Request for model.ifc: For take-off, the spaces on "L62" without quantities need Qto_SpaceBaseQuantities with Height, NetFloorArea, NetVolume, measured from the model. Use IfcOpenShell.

First a look at what the model holds.

```python
import ifcopenshell
import ifcopenshell.util.element
import ifcopenshell.util.unit

model = ifcopenshell.open("model.ifc")
print(model.schema)
for unit_type in ("LENGTHUNIT", "AREAUNIT", "VOLUMEUNIT"):
    print(unit_type, ifcopenshell.util.unit.calculate_unit_scale(model, unit_type))
storey = next(s for s in model.by_type("IfcBuildingStorey") if s.Name == "L62")
spaces = [e for e in ifcopenshell.util.element.get_decomposition(storey) if e.is_a("IfcSpace")]
for e in sorted(spaces, key=lambda e: e.id()):
    print(e.id(), e.is_a(), e.Name, list(ifcopenshell.util.element.get_psets(e, qtos_only=True)), sep=" | ")
```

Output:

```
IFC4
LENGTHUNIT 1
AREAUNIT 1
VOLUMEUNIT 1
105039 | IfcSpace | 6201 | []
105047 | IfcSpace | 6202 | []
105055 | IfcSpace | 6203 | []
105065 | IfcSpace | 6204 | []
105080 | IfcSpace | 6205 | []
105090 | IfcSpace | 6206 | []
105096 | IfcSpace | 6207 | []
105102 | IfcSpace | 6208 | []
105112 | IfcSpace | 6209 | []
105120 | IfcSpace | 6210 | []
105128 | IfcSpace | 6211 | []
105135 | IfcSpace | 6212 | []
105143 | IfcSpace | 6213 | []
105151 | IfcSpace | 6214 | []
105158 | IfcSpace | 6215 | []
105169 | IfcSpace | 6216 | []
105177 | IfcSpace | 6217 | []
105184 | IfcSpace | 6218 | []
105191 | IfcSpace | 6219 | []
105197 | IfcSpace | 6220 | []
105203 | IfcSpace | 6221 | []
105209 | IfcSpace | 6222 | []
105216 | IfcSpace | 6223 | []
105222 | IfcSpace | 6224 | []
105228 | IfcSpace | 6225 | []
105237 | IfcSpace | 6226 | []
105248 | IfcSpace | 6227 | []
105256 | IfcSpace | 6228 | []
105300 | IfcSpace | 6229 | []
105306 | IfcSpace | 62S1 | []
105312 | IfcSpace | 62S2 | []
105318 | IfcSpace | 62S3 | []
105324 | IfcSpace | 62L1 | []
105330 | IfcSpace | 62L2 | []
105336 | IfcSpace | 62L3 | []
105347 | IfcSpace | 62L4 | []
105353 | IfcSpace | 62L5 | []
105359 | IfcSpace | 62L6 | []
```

```python
import ifcopenshell
import ifcopenshell.api.pset
import ifcopenshell.geom
import ifcopenshell.util.element
import ifcopenshell.util.shape
import ifcopenshell.util.unit

model = ifcopenshell.open("model.ifc")
unit_scale = ifcopenshell.util.unit.calculate_unit_scale(model)
area_scale = ifcopenshell.util.unit.calculate_unit_scale(model, "AREAUNIT")
volume_scale = ifcopenshell.util.unit.calculate_unit_scale(model, "VOLUMEUNIT")
settings = ifcopenshell.geom.settings()

storey = next(s for s in model.by_type("IfcBuildingStorey") if s.Name == "L62")
spaces = [e for e in ifcopenshell.util.element.get_decomposition(storey) if e.is_a("IfcSpace")]

for e in sorted(spaces, key=lambda e: e.id()):
    if ifcopenshell.util.element.get_psets(e, qtos_only=True, should_inherit=False):
        continue
    # Geometry comes back in metres, in the element's own axes.
    shape = ifcopenshell.geom.create_shape(settings, e)
    values = {
        "Height": ifcopenshell.util.shape.get_z(shape.geometry) / unit_scale,
        "NetFloorArea": ifcopenshell.util.shape.get_footprint_area(shape.geometry) / area_scale,
        "NetVolume": ifcopenshell.util.shape.get_volume(shape.geometry) / volume_scale,
    }
    qto = ifcopenshell.api.pset.add_qto(model, product=e, name="Qto_SpaceBaseQuantities")
    ifcopenshell.api.pset.edit_qto(model, qto=qto, properties=values)
    print(e.id(), {k: round(v, 3) for k, v in values.items()})

model.write("model_v2.ifc")
```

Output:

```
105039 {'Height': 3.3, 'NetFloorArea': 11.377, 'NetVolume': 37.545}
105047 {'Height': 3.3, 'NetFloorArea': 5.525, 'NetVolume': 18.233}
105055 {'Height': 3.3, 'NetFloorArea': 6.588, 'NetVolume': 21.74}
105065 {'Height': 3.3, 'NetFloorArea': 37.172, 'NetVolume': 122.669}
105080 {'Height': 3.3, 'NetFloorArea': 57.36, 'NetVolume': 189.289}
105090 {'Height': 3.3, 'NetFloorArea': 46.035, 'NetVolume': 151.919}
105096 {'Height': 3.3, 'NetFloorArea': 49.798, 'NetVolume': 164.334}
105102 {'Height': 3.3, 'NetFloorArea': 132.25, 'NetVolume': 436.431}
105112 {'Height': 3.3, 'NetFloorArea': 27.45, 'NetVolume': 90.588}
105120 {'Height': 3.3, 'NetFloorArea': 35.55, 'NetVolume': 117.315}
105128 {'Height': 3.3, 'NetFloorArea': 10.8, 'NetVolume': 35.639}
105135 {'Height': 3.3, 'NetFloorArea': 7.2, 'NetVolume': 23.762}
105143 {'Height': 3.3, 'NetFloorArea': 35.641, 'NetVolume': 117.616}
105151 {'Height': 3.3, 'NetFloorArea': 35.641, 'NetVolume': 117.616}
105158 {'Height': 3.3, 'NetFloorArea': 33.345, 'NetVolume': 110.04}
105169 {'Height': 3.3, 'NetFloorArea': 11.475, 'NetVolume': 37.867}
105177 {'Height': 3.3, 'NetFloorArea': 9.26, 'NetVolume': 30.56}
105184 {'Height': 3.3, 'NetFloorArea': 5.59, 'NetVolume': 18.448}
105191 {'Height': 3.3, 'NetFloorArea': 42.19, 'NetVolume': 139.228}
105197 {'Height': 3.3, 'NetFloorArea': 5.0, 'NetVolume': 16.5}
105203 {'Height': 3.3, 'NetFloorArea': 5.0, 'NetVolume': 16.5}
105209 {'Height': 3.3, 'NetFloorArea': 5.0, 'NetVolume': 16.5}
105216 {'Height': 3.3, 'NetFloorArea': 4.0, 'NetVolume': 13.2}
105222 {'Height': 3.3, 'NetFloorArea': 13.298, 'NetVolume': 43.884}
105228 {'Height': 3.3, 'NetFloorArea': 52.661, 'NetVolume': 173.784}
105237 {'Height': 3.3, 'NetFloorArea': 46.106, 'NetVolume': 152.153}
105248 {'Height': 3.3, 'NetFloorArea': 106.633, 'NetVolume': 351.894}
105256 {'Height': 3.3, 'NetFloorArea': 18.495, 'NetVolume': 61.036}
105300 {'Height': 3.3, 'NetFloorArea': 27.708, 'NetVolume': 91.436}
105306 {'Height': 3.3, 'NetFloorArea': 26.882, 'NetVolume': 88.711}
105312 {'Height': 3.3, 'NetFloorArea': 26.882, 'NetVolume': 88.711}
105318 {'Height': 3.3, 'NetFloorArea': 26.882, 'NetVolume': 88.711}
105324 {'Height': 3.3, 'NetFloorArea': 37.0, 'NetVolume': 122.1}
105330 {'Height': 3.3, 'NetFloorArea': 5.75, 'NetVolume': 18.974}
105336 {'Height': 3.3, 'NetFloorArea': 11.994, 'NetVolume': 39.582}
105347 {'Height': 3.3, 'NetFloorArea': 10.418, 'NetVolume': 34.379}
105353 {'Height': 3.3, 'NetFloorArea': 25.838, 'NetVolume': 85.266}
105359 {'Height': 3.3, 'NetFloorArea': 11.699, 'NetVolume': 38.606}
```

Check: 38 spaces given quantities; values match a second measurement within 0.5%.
